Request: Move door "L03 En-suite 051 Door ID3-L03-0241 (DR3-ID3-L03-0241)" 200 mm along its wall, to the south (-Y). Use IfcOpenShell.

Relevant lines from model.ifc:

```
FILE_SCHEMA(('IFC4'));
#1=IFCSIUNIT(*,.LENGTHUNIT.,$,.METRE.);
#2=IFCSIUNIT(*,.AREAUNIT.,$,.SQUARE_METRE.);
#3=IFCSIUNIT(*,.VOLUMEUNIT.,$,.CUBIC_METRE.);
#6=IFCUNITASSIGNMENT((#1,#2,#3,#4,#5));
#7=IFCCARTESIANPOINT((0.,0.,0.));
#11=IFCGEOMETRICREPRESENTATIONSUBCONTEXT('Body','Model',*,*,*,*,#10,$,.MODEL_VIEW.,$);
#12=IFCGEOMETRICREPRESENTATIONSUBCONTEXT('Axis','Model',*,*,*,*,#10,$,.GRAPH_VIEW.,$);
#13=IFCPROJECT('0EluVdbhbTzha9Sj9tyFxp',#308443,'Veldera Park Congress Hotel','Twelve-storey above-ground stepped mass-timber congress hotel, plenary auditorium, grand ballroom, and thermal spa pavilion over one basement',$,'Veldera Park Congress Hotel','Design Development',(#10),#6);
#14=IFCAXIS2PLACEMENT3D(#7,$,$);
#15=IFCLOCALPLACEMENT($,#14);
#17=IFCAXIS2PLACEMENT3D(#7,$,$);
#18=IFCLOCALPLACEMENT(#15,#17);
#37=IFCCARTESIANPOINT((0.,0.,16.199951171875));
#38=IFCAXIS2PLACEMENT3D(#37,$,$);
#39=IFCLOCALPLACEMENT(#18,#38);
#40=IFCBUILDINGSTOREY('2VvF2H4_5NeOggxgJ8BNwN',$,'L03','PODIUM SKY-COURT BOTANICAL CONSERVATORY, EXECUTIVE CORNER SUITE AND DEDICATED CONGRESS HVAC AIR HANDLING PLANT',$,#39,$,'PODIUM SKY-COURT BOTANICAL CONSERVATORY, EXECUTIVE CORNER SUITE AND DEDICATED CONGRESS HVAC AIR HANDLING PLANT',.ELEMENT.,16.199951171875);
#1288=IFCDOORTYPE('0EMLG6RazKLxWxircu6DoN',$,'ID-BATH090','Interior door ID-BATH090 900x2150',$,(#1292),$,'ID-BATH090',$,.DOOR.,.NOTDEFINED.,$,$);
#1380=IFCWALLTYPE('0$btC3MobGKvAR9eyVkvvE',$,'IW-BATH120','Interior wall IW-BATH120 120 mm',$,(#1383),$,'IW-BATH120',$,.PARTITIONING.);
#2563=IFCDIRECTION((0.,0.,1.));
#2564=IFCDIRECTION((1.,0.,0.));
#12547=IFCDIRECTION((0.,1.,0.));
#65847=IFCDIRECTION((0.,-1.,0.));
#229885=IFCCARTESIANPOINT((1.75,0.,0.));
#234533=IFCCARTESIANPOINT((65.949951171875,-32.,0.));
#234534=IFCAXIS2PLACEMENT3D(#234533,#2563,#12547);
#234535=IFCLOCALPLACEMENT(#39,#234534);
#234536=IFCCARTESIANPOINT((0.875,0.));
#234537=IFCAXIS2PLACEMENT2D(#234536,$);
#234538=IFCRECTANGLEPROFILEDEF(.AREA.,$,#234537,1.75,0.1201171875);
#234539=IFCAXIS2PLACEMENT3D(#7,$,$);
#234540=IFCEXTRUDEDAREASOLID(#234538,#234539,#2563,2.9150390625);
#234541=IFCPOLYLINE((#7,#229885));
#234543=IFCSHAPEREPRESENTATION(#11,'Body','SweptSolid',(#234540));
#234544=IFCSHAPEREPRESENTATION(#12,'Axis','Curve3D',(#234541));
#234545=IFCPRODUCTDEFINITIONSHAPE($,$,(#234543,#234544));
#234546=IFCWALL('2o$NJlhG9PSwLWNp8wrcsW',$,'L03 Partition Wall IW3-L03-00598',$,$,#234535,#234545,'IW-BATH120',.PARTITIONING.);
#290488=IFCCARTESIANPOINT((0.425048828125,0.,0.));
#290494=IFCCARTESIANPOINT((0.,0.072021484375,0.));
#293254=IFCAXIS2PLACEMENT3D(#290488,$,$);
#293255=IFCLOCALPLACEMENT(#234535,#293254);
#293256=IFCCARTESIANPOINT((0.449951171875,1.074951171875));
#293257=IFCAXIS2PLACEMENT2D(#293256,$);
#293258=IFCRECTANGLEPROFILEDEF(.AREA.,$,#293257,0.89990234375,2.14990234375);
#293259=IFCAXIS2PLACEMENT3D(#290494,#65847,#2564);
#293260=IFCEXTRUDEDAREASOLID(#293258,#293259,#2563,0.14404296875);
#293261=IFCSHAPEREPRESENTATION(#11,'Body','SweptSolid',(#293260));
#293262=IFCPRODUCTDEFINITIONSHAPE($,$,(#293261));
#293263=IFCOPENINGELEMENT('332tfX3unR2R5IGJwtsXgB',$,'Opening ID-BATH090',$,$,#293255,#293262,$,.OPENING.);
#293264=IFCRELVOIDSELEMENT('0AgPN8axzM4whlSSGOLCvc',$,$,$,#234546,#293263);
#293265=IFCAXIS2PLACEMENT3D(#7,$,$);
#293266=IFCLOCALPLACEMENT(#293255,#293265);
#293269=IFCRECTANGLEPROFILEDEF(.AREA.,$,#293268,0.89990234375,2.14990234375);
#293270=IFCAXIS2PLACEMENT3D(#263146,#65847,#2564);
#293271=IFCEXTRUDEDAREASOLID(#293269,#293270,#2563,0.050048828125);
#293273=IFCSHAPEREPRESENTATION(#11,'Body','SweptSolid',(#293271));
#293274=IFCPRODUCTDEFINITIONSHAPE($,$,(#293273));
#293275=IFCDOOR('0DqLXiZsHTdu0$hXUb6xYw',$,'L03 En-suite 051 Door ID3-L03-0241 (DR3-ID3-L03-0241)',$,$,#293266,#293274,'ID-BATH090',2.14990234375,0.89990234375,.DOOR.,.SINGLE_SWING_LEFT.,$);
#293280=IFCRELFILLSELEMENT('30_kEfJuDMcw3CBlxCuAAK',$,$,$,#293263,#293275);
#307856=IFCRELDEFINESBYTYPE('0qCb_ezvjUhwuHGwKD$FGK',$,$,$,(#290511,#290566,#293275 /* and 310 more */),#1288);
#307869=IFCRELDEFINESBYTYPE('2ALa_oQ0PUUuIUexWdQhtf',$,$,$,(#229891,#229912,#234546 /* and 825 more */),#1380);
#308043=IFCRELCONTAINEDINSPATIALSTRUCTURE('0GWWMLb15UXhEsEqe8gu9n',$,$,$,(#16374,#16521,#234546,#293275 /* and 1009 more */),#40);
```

```python
import ifcopenshell
import ifcopenshell.api.geometry
import ifcopenshell.util.placement

model = ifcopenshell.open("model.ifc")

door = model.by_id(293275)
opening = door.FillsVoids[0].RelatingOpeningElement
wall = opening.VoidsElements[0].RelatingBuildingElement

wall_matrix = ifcopenshell.util.placement.get_local_placement(wall.ObjectPlacement)
shift = wall_matrix[:3, 0] * -0.2
before = ifcopenshell.util.placement.get_local_placement(door.ObjectPlacement)[:3, 3].copy()

# The door is placed relative to its opening, so it follows when the opening moves.
matrix = ifcopenshell.util.placement.get_local_placement(opening.ObjectPlacement)
matrix[:3, 3] += shift
ifcopenshell.api.geometry.edit_object_placement(
    model, product=opening, matrix=matrix, is_si=False, should_transform_children=True
)

after = ifcopenshell.util.placement.get_local_placement(door.ObjectPlacement)[:3, 3]
print("door moved by", (after - before).round(3) + 0.0)

model.write("model_updated.ifc")
```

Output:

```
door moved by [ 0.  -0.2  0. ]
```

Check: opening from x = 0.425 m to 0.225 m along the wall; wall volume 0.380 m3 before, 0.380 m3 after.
